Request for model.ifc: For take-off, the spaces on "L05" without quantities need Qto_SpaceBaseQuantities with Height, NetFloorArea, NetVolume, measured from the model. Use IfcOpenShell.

First a look at what the model holds.

```python
import ifcopenshell
import ifcopenshell.util.element
import ifcopenshell.util.unit

model = ifcopenshell.open("model.ifc")
print(model.schema)
for unit_type in ("LENGTHUNIT", "AREAUNIT", "VOLUMEUNIT"):
    print(unit_type, ifcopenshell.util.unit.calculate_unit_scale(model, unit_type))
storey = next(s for s in model.by_type("IfcBuildingStorey") if s.Name == "L05")
spaces = [e for e in ifcopenshell.util.element.get_decomposition(storey) if e.is_a("IfcSpace")]
for e in sorted(spaces, key=lambda e: e.id()):
    print(e.id(), e.is_a(), e.Name, list(ifcopenshell.util.element.get_psets(e, qtos_only=True)), sep=" | ")
```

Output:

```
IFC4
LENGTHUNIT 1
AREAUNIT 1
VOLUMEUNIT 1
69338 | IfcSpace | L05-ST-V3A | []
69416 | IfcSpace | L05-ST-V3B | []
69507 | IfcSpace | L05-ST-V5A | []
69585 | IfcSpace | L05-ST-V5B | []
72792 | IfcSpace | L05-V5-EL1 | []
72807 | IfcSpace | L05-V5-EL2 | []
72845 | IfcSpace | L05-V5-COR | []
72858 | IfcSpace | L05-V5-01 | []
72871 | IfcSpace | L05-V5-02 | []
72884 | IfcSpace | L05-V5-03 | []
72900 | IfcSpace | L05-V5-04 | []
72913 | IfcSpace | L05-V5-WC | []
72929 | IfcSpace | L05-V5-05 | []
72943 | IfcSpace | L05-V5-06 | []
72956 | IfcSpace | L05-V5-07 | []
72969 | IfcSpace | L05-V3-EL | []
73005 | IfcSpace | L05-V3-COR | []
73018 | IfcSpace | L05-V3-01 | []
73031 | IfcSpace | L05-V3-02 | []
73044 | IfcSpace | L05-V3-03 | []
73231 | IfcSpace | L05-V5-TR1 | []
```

```python
import ifcopenshell
import ifcopenshell.api.pset
import ifcopenshell.geom
import ifcopenshell.util.element
import ifcopenshell.util.shape
import ifcopenshell.util.unit

model = ifcopenshell.open("model.ifc")
unit_scale = ifcopenshell.util.unit.calculate_unit_scale(model)
area_scale = ifcopenshell.util.unit.calculate_unit_scale(model, "AREAUNIT")
volume_scale = ifcopenshell.util.unit.calculate_unit_scale(model, "VOLUMEUNIT")
settings = ifcopenshell.geom.settings()

storey = next(s for s in model.by_type("IfcBuildingStorey") if s.Name == "L05")
spaces = [e for e in ifcopenshell.util.element.get_decomposition(storey) if e.is_a("IfcSpace")]

for e in sorted(spaces, key=lambda e: e.id()):
    if ifcopenshell.util.element.get_psets(e, qtos_only=True, should_inherit=False):
        continue
    # Geometry comes back in metres, in the element's own axes.
    shape = ifcopenshell.geom.create_shape(settings, e)
    values = {
        "Height": ifcopenshell.util.shape.get_z(shape.geometry) / unit_scale,
        "NetFloorArea": ifcopenshell.util.shape.get_footprint_area(shape.geometry) / area_scale,
        "NetVolume": ifcopenshell.util.shape.get_volume(shape.geometry) / volume_scale,
    }
    qto = ifcopenshell.api.pset.add_qto(model, product=e, name="Qto_SpaceBaseQuantities")
    ifcopenshell.api.pset.edit_qto(model, qto=qto, properties=values)
    print(e.id(), {k: round(v, 3) for k, v in values.items()})

model.write("model_rev.ifc")
```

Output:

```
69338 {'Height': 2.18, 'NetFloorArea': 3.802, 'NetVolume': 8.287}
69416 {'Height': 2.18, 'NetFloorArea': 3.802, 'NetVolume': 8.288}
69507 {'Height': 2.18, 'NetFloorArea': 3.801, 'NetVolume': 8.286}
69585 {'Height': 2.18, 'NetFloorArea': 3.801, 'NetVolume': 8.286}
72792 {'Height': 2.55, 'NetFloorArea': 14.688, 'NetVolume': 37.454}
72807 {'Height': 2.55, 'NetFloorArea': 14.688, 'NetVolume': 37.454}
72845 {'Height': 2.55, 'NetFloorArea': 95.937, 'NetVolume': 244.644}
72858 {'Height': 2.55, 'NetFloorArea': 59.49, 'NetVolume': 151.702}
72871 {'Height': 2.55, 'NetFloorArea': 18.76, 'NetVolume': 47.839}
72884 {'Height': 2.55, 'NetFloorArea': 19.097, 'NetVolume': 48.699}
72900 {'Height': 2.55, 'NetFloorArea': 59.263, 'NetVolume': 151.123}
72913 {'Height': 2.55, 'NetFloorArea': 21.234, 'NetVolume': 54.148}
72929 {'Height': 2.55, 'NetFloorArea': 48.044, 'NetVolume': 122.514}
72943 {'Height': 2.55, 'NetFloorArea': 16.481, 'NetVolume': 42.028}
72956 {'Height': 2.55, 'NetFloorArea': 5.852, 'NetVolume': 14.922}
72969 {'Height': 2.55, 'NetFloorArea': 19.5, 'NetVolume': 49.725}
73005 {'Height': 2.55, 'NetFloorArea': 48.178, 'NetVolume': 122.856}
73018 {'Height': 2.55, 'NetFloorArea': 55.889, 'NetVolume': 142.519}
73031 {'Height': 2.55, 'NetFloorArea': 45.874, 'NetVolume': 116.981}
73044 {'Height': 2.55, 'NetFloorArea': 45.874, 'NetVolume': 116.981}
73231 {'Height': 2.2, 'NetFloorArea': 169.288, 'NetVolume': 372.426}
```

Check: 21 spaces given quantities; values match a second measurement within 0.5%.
